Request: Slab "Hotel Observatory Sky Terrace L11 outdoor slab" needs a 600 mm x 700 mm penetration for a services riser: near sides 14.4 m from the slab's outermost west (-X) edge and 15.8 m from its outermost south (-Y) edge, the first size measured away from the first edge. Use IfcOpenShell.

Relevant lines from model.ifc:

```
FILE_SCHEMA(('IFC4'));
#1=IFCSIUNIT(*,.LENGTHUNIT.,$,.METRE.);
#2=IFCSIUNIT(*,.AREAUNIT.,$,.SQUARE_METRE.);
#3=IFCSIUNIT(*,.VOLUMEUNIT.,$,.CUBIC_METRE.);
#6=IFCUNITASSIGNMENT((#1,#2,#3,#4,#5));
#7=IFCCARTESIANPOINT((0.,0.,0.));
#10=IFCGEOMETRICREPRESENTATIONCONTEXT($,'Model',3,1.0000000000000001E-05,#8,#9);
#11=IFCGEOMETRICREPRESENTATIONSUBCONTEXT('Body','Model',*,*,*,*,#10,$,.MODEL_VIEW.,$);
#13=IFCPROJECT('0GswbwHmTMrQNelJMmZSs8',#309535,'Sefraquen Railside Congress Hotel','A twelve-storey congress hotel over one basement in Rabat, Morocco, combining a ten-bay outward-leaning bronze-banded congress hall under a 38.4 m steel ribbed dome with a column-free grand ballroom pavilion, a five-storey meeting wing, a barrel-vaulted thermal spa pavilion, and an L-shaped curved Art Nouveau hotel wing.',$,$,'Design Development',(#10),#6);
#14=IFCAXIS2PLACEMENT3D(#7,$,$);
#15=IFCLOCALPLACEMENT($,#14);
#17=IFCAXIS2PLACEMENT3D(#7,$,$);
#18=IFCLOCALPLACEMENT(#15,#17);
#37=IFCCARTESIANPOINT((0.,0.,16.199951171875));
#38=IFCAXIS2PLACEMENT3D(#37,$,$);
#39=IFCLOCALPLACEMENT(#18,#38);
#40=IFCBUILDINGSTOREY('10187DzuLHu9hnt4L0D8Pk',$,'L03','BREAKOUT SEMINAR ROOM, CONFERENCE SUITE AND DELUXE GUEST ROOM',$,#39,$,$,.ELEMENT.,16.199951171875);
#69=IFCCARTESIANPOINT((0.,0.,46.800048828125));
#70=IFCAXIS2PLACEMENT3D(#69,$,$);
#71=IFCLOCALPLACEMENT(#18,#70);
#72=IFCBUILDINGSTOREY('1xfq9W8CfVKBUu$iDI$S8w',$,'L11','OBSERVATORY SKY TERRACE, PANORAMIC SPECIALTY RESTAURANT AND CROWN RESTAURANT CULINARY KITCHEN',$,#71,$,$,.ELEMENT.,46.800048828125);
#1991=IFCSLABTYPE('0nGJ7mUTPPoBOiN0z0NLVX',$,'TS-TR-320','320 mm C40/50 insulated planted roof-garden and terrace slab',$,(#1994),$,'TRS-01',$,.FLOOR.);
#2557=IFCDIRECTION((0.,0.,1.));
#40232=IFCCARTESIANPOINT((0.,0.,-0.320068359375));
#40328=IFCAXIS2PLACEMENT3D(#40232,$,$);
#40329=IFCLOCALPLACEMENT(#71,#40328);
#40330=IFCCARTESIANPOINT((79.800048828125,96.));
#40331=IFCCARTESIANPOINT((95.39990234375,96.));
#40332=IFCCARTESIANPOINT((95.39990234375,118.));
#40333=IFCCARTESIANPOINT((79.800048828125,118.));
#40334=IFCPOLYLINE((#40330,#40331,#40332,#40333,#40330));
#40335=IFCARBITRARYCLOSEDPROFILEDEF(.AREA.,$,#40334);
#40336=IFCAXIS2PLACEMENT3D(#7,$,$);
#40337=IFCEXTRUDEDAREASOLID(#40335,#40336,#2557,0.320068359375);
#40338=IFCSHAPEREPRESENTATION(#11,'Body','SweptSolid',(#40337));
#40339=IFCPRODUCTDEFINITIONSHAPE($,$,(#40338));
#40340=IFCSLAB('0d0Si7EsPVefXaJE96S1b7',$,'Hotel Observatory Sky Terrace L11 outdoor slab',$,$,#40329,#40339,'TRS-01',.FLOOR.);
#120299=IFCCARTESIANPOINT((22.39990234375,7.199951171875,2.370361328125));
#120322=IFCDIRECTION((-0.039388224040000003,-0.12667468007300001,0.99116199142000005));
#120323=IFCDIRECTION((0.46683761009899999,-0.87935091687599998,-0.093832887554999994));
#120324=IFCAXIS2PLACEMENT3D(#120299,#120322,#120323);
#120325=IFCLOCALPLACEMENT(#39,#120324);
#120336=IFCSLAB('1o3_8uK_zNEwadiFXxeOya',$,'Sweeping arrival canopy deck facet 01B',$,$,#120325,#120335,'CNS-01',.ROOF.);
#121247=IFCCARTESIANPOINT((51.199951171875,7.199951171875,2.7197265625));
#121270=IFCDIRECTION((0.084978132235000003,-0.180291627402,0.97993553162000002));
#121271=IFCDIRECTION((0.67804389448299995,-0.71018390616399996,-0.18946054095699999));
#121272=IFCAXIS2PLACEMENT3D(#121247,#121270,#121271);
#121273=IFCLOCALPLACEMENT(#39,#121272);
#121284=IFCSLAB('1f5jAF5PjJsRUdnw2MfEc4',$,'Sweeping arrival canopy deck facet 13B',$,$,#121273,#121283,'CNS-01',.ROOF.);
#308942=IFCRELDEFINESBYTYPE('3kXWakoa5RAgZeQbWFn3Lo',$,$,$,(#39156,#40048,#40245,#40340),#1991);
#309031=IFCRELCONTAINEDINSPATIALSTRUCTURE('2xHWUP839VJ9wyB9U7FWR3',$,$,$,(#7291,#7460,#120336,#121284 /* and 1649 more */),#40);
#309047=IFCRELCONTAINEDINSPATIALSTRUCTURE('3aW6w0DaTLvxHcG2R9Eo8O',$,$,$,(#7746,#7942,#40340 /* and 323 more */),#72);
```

```python
import numpy as np
import ifcopenshell
import ifcopenshell.api.feature
import ifcopenshell.api.geometry
import ifcopenshell.api.root
import ifcopenshell.geom
import ifcopenshell.util.placement
import ifcopenshell.util.representation
import ifcopenshell.util.shape
import ifcopenshell.util.unit

model = ifcopenshell.open("model.ifc")
unit_scale = ifcopenshell.util.unit.calculate_unit_scale(model)
settings = ifcopenshell.geom.settings()


def volume(element):
    """Net volume in cubic metres, openings subtracted."""
    shape = ifcopenshell.geom.create_shape(settings, element)
    return ifcopenshell.util.shape.get_volume(shape.geometry)


slab = model.by_guid("0d0Si7EsPVefXaJE96S1b7")
before = volume(slab)

# Extent in the slab's own axes, in metres. The edges named are its -X and -Y sides.
slab_shape = ifcopenshell.geom.create_shape(settings, slab)
vertices = ifcopenshell.util.shape.get_vertices(slab_shape.geometry)
x_min, y_min, bottom = vertices.min(axis=0)
top = vertices[:, 2].max()

opening = ifcopenshell.api.root.create_entity(model, ifc_class="IfcOpeningElement", name="Services riser opening", predefined_type="OPENING")
context = ifcopenshell.util.representation.get_context(model, "Model", "Body", "MODEL_VIEW")
width, depth = 0.6, 0.7
outline = [(0.0, 0.0), (width, 0.0), (width, depth), (0.0, depth), (0.0, 0.0)]
# Overshoot both faces by 50 mm so the cut is clean.
shape = ifcopenshell.api.geometry.add_slab_representation(
    model, context=context, depth=top - bottom + 0.1, polyline=outline
)
ifcopenshell.api.geometry.assign_representation(model, product=opening, representation=shape)

matrix = ifcopenshell.util.placement.get_local_placement(slab.ObjectPlacement)
matrix[:, 3] = matrix @ np.append(np.array([x_min + 14.4, y_min + 15.8, bottom - 0.05]) / unit_scale, 1.0)
ifcopenshell.api.geometry.edit_object_placement(model, product=opening, matrix=matrix, is_si=False)
ifcopenshell.api.feature.add_feature(model, feature=opening, element=slab)

after = volume(slab)

print(f"slab volume {before:.3f} -> {after:.3f} m3")

model.write("model_rev.ifc")
```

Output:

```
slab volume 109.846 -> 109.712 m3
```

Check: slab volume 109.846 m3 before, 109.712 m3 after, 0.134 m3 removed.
